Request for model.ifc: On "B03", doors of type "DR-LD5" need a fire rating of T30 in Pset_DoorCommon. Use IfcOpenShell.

First a look at what the model holds.

```python
import ifcopenshell
import ifcopenshell.util.element

model = ifcopenshell.open("model.ifc")
print(model.schema)
storey = next(s for s in model.by_type("IfcBuildingStorey") if s.Name == "B03")
doors = [e for e in ifcopenshell.util.element.get_decomposition(storey) if e.is_a("IfcDoor")]
seen = {}
for e in doors:
    element_type = ifcopenshell.util.element.get_type(e)
    key = (element_type.Name if element_type != e and element_type else None, ifcopenshell.util.element.get_pset(e, "Pset_DoorCommon", "FireRating"))
    seen[key] = seen.get(key, 0) + 1
for (name, value), count in sorted(seen.items(), key=str):
    print(count, "x", name, "|", value)
```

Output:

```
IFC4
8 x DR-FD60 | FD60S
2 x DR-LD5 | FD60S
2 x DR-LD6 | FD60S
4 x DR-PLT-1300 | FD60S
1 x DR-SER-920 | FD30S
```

```python
import ifcopenshell
import ifcopenshell.api.pset
import ifcopenshell.util.element

model = ifcopenshell.open("model.ifc")

storey = next(s for s in model.by_type("IfcBuildingStorey") if s.Name == "B03")
doors = [e for e in ifcopenshell.util.element.get_decomposition(storey) if e.is_a("IfcDoor")]

count = 0
for e in doors:
    element_type = ifcopenshell.util.element.get_type(e)
    if element_type in (None, e) or element_type.Name != "DR-LD5":
        continue
    found = ifcopenshell.util.element.get_pset(e, "Pset_DoorCommon", should_inherit=False)
    if found:
        pset = model.by_id(found["id"])
        if len(ifcopenshell.util.element.get_elements_by_pset(pset)) > 1:
            pset = ifcopenshell.api.pset.unshare_pset(model, products=[e], pset=pset)[0]
    else:
        pset = ifcopenshell.api.pset.add_pset(model, product=e, name="Pset_DoorCommon")
    ifcopenshell.api.pset.edit_pset(model, pset=pset, properties={"FireRating": "T30"})
    count += 1

print(count, "doors updated")

model.write("model_updated.ifc")
```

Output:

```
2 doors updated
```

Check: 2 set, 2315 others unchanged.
